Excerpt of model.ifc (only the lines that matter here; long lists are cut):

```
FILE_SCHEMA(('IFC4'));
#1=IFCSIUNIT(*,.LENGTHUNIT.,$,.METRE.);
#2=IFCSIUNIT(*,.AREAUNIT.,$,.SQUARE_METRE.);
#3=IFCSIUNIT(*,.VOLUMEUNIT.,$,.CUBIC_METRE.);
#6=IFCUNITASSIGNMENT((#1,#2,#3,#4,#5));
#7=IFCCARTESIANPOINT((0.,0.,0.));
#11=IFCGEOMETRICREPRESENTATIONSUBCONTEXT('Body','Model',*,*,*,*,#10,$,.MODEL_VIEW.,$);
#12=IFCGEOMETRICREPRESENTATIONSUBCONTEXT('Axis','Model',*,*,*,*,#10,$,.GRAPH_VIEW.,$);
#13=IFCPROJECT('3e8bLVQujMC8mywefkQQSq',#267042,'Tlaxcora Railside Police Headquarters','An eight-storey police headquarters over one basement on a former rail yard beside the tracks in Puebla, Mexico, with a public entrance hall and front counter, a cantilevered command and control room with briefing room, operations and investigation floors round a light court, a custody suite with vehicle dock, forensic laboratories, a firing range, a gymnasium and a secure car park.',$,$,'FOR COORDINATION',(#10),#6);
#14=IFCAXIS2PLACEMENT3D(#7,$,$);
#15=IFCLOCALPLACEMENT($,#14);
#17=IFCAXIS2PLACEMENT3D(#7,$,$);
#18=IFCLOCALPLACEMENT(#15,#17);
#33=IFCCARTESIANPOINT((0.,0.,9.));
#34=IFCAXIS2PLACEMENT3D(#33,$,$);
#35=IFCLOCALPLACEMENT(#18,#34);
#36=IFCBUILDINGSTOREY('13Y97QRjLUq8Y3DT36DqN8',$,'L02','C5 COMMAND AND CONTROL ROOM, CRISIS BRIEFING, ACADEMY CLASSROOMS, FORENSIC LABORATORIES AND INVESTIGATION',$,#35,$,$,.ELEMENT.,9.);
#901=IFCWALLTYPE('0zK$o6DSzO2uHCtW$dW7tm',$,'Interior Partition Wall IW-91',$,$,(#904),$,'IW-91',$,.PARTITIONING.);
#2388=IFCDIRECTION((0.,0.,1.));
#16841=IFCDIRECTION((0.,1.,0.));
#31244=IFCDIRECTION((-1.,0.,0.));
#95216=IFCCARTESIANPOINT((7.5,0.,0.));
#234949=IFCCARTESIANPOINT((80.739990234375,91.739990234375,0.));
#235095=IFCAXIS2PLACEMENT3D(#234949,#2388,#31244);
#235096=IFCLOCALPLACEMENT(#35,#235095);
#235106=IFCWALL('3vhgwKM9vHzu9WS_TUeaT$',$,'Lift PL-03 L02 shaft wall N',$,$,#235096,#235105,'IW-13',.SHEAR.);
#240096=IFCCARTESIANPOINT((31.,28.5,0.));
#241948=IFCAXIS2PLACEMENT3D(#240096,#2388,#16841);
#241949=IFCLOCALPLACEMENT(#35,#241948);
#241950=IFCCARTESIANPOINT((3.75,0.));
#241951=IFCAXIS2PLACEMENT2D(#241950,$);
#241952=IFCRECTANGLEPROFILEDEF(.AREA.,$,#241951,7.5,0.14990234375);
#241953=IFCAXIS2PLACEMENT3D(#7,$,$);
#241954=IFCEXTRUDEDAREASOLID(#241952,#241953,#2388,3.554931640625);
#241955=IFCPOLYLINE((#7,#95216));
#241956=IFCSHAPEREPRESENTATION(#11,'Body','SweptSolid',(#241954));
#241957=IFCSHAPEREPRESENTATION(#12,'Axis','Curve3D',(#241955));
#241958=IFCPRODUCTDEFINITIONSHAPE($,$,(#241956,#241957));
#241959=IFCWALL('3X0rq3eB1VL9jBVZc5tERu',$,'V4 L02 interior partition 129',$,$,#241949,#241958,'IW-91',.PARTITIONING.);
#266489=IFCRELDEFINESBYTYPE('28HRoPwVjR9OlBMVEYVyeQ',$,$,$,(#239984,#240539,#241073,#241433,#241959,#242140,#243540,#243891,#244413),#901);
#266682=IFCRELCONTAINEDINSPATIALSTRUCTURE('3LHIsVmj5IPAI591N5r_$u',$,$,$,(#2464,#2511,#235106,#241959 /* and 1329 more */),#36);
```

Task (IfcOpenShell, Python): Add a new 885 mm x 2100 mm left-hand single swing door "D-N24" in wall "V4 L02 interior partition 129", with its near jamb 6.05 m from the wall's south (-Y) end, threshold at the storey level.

```python
import numpy as np
import ifcopenshell
import ifcopenshell.api.feature
import ifcopenshell.api.geometry
import ifcopenshell.api.root
import ifcopenshell.api.spatial
import ifcopenshell.geom
import ifcopenshell.util.element
import ifcopenshell.util.placement
import ifcopenshell.util.representation
import ifcopenshell.util.shape
import ifcopenshell.util.unit

model = ifcopenshell.open("model.ifc")
unit_scale = ifcopenshell.util.unit.calculate_unit_scale(model)
settings = ifcopenshell.geom.settings()


def volume(element):
    """Net volume in cubic metres, openings subtracted."""
    shape = ifcopenshell.geom.create_shape(settings, element)
    return ifcopenshell.util.shape.get_volume(shape.geometry)


wall = model.by_guid("3X0rq3eB1VL9jBVZc5tERu")
storey = ifcopenshell.util.element.get_container(wall, ifc_class="IfcBuildingStorey")
context = ifcopenshell.util.representation.get_context(model, "Model", "Body", "MODEL_VIEW")
before = volume(wall)

width, height, from_end, sill = 0.885, 2.1, 6.05, 0.0  # metres

# The wall runs along its own X axis, and the end named is its -X end.
wall_shape = ifcopenshell.geom.create_shape(settings, wall)
x, y, z = ifcopenshell.util.shape.get_vertices(wall_shape.geometry).T
start = x.min() + from_end
face, thickness = float(y.min()), float(y.max() - y.min())
wall_matrix = ifcopenshell.util.placement.get_local_placement(wall.ObjectPlacement)
level = ifcopenshell.util.placement.get_local_placement(storey.ObjectPlacement)[2, 3]


def in_wall(x, y):
    """Placement at x, y metres in the wall's axes, at sill height."""
    matrix = wall_matrix.copy()
    matrix[:, 3] = wall_matrix @ np.array([x / unit_scale, y / unit_scale, 0.0, 1.0])
    matrix[2, 3] = level + sill / unit_scale
    return matrix


# Opening: a box that overshoots both wall faces by 50 mm.
opening = ifcopenshell.api.root.create_entity(model, ifc_class="IfcOpeningElement", predefined_type="OPENING")
box = ifcopenshell.api.geometry.add_wall_representation(
    model, context=context, length=width, height=height, thickness=thickness + 0.1
)
ifcopenshell.api.geometry.assign_representation(model, product=opening, representation=box)
ifcopenshell.api.geometry.edit_object_placement(model, product=opening, matrix=in_wall(start, face - 0.05), is_si=False)
ifcopenshell.api.feature.add_feature(model, feature=opening, element=wall)

door = ifcopenshell.api.root.create_entity(model, ifc_class="IfcDoor", name="D-N24", predefined_type="DOOR")
door.OverallWidth, door.OverallHeight = width / unit_scale, height / unit_scale
door.OperationType = "SINGLE_SWING_LEFT"
body = ifcopenshell.api.geometry.add_door_representation(
    model,
    context=context,
    overall_width=door.OverallWidth,
    overall_height=door.OverallHeight,
    operation_type="SINGLE_SWING_LEFT",
    lining_properties={"LiningDepth": thickness / unit_scale, "ThresholdDepth": thickness / unit_scale},
)
ifcopenshell.api.geometry.assign_representation(model, product=door, representation=body)
ifcopenshell.api.spatial.assign_container(model, products=[door], relating_structure=storey)
ifcopenshell.api.feature.add_filling(model, opening=opening, element=door)

# The lining spans the wall, so the door starts at the wall face.
ifcopenshell.api.geometry.edit_object_placement(model, product=door, matrix=in_wall(start, face), is_si=False)

after = volume(wall)

print(f"wall volume {before:.3f} -> {after:.3f} m3")

model.write("model_v2.ifc")
```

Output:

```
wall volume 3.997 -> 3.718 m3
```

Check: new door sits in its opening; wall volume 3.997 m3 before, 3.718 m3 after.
